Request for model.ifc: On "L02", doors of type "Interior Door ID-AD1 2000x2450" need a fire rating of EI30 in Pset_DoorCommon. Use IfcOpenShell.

First a look at what the model holds.

```python
import ifcopenshell
import ifcopenshell.util.element

model = ifcopenshell.open("model.ifc")
print(model.schema)
storey = next(s for s in model.by_type("IfcBuildingStorey") if s.Name == "L02")
doors = [e for e in ifcopenshell.util.element.get_decomposition(storey) if e.is_a("IfcDoor")]
seen = {}
for e in doors:
    element_type = ifcopenshell.util.element.get_type(e)
    key = (element_type.Name if element_type != e and element_type else None, ifcopenshell.util.element.get_pset(e, "Pset_DoorCommon", "FireRating"))
    seen[key] = seen.get(key, 0) + 1
for (name, value), count in sorted(seen.items(), key=str):
    print(count, "x", name, "|", value)
```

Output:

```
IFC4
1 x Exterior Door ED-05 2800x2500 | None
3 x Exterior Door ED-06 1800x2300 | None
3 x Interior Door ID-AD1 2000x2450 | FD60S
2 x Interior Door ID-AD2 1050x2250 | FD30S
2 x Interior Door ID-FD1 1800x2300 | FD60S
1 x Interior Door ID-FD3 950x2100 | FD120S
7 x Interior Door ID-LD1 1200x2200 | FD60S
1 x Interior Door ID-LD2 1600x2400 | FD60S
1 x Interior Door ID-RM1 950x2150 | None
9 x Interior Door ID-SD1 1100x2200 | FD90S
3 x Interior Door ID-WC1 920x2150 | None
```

```python
import ifcopenshell
import ifcopenshell.api.pset
import ifcopenshell.util.element

model = ifcopenshell.open("model.ifc")

storey = next(s for s in model.by_type("IfcBuildingStorey") if s.Name == "L02")
doors = [e for e in ifcopenshell.util.element.get_decomposition(storey) if e.is_a("IfcDoor")]

count = 0
for e in doors:
    element_type = ifcopenshell.util.element.get_type(e)
    if element_type in (None, e) or element_type.Name != "Interior Door ID-AD1 2000x2450":
        continue
    # add_pset returns the element's existing set when there is one.
    pset = ifcopenshell.api.pset.add_pset(model, product=e, name="Pset_DoorCommon")
    ifcopenshell.api.pset.edit_pset(model, pset=pset, properties={"FireRating": "EI30"})
    count += 1

print(count, "doors updated")

model.write("model_rev.ifc")
```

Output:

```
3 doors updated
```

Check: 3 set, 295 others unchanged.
